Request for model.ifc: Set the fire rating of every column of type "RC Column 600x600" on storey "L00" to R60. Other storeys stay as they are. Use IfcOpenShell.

First a look at what the model holds.

```python
import ifcopenshell
import ifcopenshell.util.element

model = ifcopenshell.open("model.ifc")
print(model.schema)
storey = next(s for s in model.by_type("IfcBuildingStorey") if s.Name == "L00")
columns = [e for e in ifcopenshell.util.element.get_decomposition(storey) if e.is_a("IfcColumn")]
seen = {}
for e in columns:
    element_type = ifcopenshell.util.element.get_type(e)
    key = (element_type.Name if element_type != e and element_type else None, ifcopenshell.util.element.get_pset(e, "Pset_ColumnCommon", "FireRating"))
    seen[key] = seen.get(key, 0) + 1
for (name, value), count in sorted(seen.items(), key=str):
    print(count, "x", name, "|", value)
```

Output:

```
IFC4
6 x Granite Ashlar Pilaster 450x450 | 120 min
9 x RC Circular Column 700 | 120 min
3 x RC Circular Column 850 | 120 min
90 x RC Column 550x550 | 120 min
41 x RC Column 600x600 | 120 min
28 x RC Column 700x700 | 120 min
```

```python
import ifcopenshell
import ifcopenshell.api.pset
import ifcopenshell.util.element

model = ifcopenshell.open("model.ifc")

storey = next(s for s in model.by_type("IfcBuildingStorey") if s.Name == "L00")
columns = [e for e in ifcopenshell.util.element.get_decomposition(storey) if e.is_a("IfcColumn")]

count = 0
for e in columns:
    element_type = ifcopenshell.util.element.get_type(e)
    if element_type in (None, e) or element_type.Name != "RC Column 600x600":
        continue
    # add_pset returns the element's existing set when there is one.
    pset = ifcopenshell.api.pset.add_pset(model, product=e, name="Pset_ColumnCommon")
    ifcopenshell.api.pset.edit_pset(model, pset=pset, properties={"FireRating": "R60"})
    count += 1

print(count, "columns updated")

model.write("model_v2.ifc")
```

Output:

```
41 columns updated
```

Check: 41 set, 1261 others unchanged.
